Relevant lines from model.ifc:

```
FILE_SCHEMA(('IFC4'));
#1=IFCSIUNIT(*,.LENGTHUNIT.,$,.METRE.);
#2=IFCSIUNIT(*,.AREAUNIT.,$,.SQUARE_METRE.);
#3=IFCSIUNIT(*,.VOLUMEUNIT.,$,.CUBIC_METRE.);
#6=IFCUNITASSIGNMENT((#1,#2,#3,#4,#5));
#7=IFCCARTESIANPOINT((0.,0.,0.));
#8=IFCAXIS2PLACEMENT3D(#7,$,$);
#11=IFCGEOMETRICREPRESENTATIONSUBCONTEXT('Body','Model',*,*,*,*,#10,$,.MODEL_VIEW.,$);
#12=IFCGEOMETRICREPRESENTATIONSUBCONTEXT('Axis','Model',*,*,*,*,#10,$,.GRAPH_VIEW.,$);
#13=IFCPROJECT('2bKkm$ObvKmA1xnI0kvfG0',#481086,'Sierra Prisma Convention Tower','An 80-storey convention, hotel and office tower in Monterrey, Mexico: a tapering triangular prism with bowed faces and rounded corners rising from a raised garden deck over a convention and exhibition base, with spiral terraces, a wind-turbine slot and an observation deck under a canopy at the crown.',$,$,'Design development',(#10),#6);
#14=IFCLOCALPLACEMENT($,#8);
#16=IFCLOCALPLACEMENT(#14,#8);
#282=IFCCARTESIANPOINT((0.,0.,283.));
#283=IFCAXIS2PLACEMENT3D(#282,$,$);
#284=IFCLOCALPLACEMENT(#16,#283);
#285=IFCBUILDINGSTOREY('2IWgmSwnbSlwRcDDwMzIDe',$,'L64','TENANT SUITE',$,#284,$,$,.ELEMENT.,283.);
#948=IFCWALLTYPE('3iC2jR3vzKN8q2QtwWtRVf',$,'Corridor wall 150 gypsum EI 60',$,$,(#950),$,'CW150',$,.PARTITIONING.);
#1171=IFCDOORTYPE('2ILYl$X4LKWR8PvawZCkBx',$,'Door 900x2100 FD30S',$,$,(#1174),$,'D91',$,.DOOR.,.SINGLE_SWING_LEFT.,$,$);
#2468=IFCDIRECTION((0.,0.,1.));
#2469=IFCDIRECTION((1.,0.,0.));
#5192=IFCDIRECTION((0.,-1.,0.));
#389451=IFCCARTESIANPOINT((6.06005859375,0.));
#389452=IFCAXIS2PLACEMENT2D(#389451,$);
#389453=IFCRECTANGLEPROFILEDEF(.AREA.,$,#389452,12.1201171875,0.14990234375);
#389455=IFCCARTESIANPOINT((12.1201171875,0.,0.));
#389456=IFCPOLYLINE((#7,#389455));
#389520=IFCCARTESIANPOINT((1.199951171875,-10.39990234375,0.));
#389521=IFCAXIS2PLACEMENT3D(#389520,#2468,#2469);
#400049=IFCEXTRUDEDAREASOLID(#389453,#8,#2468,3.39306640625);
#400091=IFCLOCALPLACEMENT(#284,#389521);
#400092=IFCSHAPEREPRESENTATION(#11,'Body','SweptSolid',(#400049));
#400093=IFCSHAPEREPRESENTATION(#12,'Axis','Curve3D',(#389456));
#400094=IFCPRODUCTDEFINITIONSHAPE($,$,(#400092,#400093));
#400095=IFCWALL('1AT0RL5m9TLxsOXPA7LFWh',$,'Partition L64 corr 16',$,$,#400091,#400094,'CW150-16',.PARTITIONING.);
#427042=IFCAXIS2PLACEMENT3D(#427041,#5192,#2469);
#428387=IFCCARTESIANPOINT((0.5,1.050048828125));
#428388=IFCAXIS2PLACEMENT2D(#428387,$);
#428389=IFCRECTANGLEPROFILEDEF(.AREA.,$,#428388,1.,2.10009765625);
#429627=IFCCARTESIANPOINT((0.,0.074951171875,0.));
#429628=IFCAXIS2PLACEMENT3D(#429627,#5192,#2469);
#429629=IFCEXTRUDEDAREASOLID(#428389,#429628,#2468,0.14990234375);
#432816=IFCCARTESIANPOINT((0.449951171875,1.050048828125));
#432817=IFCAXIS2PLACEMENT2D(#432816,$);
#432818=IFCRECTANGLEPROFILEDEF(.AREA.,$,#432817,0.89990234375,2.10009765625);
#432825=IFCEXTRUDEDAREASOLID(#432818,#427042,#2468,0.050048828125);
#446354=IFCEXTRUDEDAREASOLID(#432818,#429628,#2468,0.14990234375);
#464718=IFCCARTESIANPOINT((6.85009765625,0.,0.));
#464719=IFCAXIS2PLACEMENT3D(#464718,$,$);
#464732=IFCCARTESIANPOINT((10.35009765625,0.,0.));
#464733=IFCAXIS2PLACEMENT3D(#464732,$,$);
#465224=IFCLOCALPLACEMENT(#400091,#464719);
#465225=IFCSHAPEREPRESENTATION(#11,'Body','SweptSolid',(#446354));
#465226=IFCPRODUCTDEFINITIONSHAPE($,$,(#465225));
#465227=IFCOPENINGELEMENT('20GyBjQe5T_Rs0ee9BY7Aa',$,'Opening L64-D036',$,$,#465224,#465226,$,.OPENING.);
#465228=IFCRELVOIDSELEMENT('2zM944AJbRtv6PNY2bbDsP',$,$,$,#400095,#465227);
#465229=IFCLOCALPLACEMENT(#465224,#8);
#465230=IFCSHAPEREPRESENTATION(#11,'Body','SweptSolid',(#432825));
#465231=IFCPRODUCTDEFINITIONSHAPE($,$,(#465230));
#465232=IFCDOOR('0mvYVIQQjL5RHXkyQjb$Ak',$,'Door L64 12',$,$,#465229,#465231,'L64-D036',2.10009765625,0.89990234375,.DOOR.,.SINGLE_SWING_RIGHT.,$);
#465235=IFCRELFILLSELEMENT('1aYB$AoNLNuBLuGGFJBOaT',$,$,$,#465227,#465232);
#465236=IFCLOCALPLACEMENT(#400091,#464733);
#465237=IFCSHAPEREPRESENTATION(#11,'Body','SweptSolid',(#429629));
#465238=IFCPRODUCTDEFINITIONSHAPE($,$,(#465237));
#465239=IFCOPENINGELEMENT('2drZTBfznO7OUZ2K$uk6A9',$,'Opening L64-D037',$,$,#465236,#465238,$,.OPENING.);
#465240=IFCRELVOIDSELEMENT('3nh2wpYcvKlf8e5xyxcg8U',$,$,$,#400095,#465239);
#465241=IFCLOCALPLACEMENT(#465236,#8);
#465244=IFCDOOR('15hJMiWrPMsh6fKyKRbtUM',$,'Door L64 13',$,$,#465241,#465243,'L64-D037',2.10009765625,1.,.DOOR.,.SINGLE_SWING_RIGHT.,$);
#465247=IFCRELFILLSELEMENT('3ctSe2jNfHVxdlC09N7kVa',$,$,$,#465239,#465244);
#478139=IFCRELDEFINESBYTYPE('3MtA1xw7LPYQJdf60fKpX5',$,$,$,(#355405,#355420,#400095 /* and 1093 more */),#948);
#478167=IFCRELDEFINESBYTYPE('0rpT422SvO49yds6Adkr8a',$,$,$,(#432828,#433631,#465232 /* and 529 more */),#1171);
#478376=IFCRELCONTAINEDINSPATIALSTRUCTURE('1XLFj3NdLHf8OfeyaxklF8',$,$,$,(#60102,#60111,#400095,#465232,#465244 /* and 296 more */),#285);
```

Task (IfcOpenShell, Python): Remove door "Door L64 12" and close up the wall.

```python
import ifcopenshell
import ifcopenshell.api.feature
import ifcopenshell.api.root
import ifcopenshell.geom
import ifcopenshell.util.shape

model = ifcopenshell.open("model.ifc")
settings = ifcopenshell.geom.settings()


def volume(element):
    """Net volume in cubic metres, openings subtracted."""
    shape = ifcopenshell.geom.create_shape(settings, element)
    return ifcopenshell.util.shape.get_volume(shape.geometry)


door = model.by_guid("0mvYVIQQjL5RHXkyQjb$Ak")
opening = door.FillsVoids[0].RelatingOpeningElement
wall = opening.VoidsElements[0].RelatingBuildingElement
before = volume(wall)

ifcopenshell.api.root.remove_product(model, product=door)
ifcopenshell.api.feature.remove_feature(model, feature=opening)

after = volume(wall)

print(f"wall volume {before:.3f} -> {after:.3f} m3")

model.write("model-out.ifc")
```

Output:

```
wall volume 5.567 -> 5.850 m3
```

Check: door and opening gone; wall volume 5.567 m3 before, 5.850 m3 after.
